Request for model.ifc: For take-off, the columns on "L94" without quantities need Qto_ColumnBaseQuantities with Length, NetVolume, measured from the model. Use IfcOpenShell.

First a look at what the model holds.

```python
import ifcopenshell
import ifcopenshell.util.element
import ifcopenshell.util.unit

model = ifcopenshell.open("model.ifc")
print(model.schema)
for unit_type in ("LENGTHUNIT", "AREAUNIT", "VOLUMEUNIT"):
    print(unit_type, ifcopenshell.util.unit.calculate_unit_scale(model, unit_type))
storey = next(s for s in model.by_type("IfcBuildingStorey") if s.Name == "L94")
columns = [e for e in ifcopenshell.util.element.get_decomposition(storey) if e.is_a("IfcColumn")]
for e in sorted(columns, key=lambda e: e.id()):
    print(e.id(), e.is_a(), e.Name, list(ifcopenshell.util.element.get_psets(e, qtos_only=True)), sep=" | ")
```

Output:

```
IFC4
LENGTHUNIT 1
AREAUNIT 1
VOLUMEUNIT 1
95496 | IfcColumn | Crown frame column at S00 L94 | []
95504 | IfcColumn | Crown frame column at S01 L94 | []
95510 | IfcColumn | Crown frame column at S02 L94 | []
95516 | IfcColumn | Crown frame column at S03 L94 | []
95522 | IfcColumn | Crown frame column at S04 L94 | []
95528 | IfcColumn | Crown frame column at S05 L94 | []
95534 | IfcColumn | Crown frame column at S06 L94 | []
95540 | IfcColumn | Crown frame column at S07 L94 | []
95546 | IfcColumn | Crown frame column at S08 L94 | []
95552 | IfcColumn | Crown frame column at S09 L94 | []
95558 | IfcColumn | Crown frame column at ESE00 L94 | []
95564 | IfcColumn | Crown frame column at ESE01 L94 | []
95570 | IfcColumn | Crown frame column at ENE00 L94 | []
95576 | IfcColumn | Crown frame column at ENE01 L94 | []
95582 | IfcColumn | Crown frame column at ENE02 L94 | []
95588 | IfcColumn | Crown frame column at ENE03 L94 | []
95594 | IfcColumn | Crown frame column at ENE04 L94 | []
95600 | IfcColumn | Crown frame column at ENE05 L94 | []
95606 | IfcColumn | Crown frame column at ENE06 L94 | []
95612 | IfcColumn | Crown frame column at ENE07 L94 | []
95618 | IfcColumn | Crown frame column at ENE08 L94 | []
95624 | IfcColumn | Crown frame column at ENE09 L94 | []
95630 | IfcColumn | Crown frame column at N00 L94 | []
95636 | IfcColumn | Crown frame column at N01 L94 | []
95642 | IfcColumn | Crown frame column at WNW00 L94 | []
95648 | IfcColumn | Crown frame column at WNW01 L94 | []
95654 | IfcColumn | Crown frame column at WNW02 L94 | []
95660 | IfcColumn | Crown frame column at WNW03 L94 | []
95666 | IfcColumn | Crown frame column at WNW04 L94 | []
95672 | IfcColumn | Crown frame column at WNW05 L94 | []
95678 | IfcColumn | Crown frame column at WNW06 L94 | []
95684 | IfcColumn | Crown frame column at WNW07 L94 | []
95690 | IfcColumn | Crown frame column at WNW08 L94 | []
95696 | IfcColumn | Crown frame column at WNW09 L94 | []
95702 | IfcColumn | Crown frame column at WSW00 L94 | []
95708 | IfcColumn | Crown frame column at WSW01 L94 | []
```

```python
import ifcopenshell
import ifcopenshell.api.pset
import ifcopenshell.geom
import ifcopenshell.util.element
import ifcopenshell.util.shape
import ifcopenshell.util.unit

model = ifcopenshell.open("model.ifc")
unit_scale = ifcopenshell.util.unit.calculate_unit_scale(model)
volume_scale = ifcopenshell.util.unit.calculate_unit_scale(model, "VOLUMEUNIT")
settings = ifcopenshell.geom.settings()

storey = next(s for s in model.by_type("IfcBuildingStorey") if s.Name == "L94")
columns = [e for e in ifcopenshell.util.element.get_decomposition(storey) if e.is_a("IfcColumn")]

for e in sorted(columns, key=lambda e: e.id()):
    if ifcopenshell.util.element.get_psets(e, qtos_only=True, should_inherit=False):
        continue
    # Geometry comes back in metres, in the element's own axes.
    shape = ifcopenshell.geom.create_shape(settings, e)
    values = {
        "Length": ifcopenshell.util.shape.get_z(shape.geometry) / unit_scale,
        "NetVolume": ifcopenshell.util.shape.get_volume(shape.geometry) / volume_scale,
    }
    qto = ifcopenshell.api.pset.add_qto(model, product=e, name="Qto_ColumnBaseQuantities")
    ifcopenshell.api.pset.edit_qto(model, qto=qto, properties=values)
    print(e.id(), {k: round(v, 3) for k, v in values.items()})

model.write("model_rev.ifc")
```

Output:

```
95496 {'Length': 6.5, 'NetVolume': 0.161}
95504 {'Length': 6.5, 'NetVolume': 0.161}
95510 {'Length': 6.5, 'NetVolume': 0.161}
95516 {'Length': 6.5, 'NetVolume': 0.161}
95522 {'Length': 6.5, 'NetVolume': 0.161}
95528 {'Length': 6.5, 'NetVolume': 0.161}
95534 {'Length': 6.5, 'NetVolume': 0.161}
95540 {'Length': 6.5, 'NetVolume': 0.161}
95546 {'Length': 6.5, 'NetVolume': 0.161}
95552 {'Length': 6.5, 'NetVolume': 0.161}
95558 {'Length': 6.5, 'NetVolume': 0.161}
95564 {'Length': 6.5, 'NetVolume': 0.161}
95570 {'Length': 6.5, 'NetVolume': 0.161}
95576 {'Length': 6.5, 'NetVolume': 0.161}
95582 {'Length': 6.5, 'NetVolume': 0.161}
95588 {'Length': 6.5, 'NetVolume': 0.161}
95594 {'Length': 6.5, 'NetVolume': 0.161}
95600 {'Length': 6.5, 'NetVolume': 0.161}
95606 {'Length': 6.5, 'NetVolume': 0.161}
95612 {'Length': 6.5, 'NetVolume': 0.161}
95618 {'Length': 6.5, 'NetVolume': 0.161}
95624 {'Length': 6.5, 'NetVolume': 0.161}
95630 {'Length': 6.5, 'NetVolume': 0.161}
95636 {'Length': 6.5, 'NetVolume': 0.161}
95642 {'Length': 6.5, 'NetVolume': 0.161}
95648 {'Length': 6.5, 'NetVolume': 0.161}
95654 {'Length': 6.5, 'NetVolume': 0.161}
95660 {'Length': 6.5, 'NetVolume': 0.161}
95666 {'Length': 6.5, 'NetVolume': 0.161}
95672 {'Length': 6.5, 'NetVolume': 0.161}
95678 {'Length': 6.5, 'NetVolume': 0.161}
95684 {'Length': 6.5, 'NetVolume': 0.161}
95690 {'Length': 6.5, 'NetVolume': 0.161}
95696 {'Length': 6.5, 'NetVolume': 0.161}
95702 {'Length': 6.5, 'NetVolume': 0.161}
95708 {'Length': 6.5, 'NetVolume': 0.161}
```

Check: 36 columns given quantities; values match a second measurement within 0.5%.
